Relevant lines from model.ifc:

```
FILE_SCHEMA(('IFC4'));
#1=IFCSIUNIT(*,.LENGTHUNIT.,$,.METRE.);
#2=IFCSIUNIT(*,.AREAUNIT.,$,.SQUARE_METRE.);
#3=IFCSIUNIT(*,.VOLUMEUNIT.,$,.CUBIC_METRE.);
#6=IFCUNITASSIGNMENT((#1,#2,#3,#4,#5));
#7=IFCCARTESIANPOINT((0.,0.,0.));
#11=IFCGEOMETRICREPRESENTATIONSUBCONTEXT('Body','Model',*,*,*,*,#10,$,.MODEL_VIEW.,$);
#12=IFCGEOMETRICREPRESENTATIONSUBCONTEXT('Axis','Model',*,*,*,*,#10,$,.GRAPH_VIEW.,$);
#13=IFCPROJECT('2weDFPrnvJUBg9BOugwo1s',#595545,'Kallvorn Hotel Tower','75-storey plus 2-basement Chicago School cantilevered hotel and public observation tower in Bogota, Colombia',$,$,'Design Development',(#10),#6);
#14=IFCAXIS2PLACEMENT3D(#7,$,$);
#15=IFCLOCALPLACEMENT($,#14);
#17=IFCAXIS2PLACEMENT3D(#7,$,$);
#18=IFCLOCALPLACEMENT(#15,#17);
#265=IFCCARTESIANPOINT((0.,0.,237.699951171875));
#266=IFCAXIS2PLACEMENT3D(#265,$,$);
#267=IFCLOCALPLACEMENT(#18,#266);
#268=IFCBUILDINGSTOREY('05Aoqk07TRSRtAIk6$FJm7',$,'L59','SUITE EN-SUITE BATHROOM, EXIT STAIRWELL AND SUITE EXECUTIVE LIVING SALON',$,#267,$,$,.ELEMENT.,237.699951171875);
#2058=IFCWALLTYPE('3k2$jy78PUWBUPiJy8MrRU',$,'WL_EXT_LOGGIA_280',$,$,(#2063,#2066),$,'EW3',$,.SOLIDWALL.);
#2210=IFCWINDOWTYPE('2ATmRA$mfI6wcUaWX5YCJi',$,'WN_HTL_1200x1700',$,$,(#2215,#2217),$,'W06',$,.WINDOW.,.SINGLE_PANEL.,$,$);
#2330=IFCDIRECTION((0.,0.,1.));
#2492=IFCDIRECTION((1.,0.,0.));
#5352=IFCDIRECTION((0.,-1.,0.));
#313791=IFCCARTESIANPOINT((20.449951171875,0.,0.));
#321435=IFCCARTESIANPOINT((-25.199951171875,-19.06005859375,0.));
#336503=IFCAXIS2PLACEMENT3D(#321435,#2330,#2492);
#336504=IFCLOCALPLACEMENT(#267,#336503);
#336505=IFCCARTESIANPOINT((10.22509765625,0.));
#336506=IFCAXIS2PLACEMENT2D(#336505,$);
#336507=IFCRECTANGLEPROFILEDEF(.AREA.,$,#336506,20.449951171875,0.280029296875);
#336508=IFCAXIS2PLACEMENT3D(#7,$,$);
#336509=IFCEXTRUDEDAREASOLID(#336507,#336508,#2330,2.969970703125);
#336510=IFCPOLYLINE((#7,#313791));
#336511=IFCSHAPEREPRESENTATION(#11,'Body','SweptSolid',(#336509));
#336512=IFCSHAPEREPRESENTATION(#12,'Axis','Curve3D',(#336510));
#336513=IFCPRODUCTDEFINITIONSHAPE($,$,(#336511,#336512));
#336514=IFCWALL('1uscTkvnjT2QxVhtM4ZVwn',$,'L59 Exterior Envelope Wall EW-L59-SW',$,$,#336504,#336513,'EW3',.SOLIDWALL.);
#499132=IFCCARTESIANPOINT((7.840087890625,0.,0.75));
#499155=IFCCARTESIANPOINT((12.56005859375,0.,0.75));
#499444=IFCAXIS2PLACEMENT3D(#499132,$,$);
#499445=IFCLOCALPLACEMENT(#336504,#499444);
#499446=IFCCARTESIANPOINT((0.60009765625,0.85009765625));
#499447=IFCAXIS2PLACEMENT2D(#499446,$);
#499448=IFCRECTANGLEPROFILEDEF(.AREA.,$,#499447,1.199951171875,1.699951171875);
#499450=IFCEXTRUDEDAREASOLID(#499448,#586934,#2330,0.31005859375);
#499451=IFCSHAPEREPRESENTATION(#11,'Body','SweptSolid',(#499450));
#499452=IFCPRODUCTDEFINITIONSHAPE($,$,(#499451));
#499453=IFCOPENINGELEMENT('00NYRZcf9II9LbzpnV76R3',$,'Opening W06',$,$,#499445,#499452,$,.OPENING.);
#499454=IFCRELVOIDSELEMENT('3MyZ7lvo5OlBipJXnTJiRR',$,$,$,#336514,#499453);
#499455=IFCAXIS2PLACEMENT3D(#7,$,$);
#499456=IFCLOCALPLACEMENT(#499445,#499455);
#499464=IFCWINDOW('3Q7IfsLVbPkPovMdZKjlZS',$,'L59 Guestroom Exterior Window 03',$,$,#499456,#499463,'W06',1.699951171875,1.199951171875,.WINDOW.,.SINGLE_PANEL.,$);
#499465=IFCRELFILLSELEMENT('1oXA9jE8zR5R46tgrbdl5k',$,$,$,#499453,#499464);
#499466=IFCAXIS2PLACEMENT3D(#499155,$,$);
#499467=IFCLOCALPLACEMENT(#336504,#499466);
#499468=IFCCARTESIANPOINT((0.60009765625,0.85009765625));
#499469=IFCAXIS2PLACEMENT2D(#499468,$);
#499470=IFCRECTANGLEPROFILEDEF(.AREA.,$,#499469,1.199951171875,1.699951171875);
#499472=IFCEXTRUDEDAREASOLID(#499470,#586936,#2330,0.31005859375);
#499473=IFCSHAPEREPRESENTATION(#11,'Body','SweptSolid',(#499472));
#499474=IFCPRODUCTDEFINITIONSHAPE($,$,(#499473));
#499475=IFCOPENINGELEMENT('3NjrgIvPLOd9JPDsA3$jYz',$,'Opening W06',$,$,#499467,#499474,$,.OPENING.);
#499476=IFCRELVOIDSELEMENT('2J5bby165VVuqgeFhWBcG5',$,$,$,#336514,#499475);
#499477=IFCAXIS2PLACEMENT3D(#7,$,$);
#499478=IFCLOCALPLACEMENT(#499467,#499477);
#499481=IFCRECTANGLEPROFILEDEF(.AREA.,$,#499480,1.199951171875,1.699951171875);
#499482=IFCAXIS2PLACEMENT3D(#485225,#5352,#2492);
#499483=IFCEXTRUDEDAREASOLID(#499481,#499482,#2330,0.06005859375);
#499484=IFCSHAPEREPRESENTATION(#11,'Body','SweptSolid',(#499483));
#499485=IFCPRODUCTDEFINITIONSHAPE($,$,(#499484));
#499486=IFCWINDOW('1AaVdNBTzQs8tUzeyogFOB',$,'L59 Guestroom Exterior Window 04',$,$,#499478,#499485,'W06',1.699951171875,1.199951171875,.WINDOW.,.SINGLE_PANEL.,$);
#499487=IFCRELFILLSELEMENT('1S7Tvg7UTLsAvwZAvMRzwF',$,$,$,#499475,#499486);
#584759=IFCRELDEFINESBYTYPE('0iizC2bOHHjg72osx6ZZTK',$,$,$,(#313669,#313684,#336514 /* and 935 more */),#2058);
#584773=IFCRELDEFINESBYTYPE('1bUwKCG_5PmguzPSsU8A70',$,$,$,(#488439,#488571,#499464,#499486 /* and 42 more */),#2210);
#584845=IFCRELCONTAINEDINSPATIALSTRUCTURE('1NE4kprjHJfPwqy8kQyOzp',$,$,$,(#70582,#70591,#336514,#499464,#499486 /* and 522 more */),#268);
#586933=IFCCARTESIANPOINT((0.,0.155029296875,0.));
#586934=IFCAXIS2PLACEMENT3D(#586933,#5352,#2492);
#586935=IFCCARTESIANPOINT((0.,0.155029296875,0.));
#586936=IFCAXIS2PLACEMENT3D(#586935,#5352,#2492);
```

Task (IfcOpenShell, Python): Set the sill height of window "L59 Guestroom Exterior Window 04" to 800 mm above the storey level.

```python
import numpy as np
import ifcopenshell
import ifcopenshell.api.geometry
import ifcopenshell.geom
import ifcopenshell.util.element
import ifcopenshell.util.placement
import ifcopenshell.util.shape
import ifcopenshell.util.unit

model = ifcopenshell.open("model.ifc")
unit_scale = ifcopenshell.util.unit.calculate_unit_scale(model)

window = model.by_id(499486)
opening = window.FillsVoids[0].RelatingOpeningElement
storey = ifcopenshell.util.element.get_container(window, ifc_class="IfcBuildingStorey")
level = ifcopenshell.util.placement.get_local_placement(storey.ObjectPlacement)[2, 3]

# The opening's origin need not be at the sill, so measure its lowest point.
shape = ifcopenshell.geom.create_shape(ifcopenshell.geom.settings(), opening)
bottom = ifcopenshell.util.shape.get_shape_bottom_elevation(shape, shape.geometry) / unit_scale
dz = level + 0.8 / unit_scale - bottom

shift = np.array([0.0, 0.0, dz])
# The window is placed relative to its opening, so it follows when the opening moves.
matrix = ifcopenshell.util.placement.get_local_placement(opening.ObjectPlacement)
matrix[:3, 3] += shift
ifcopenshell.api.geometry.edit_object_placement(
    model, product=opening, matrix=matrix, is_si=False, should_transform_children=True
)

print(f"moved by {dz * unit_scale:+.3f} m")

model.write("model_rev.ifc")
```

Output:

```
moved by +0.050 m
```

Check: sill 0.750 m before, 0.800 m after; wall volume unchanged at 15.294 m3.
